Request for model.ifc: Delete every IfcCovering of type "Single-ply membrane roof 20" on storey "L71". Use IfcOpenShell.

First a look at what the model holds.

```python
import ifcopenshell
import ifcopenshell.util.element

model = ifcopenshell.open("model.ifc")
print(model.schema)
storey = next(s for s in model.by_type("IfcBuildingStorey") if s.Name == "L71")
coverings = [e for e in ifcopenshell.util.element.get_decomposition(storey) if e.is_a("IfcCovering")]
seen = {}
for e in coverings:
    element_type = ifcopenshell.util.element.get_type(e)
    name = element_type.Name if element_type not in (None, e) else None
    seen[name] = seen.get(name, 0) + 1
for name, count in sorted(seen.items(), key=str):
    print(count, "x", name)
```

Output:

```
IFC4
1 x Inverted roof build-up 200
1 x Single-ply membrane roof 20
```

```python
import ifcopenshell
import ifcopenshell.api.root
import ifcopenshell.util.element

model = ifcopenshell.open("model.ifc")

storey = next(s for s in model.by_type("IfcBuildingStorey") if s.Name == "L71")
coverings = [e for e in ifcopenshell.util.element.get_decomposition(storey) if e.is_a("IfcCovering")]
targets = [e for e in coverings if (t := ifcopenshell.util.element.get_type(e)) not in (None, e) and t.Name == "Single-ply membrane roof 20"]

for e in targets:
    ifcopenshell.api.root.remove_product(model, product=e)
print(len(targets), "removed")

model.write("model_v2.ifc")
```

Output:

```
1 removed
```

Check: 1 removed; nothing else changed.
